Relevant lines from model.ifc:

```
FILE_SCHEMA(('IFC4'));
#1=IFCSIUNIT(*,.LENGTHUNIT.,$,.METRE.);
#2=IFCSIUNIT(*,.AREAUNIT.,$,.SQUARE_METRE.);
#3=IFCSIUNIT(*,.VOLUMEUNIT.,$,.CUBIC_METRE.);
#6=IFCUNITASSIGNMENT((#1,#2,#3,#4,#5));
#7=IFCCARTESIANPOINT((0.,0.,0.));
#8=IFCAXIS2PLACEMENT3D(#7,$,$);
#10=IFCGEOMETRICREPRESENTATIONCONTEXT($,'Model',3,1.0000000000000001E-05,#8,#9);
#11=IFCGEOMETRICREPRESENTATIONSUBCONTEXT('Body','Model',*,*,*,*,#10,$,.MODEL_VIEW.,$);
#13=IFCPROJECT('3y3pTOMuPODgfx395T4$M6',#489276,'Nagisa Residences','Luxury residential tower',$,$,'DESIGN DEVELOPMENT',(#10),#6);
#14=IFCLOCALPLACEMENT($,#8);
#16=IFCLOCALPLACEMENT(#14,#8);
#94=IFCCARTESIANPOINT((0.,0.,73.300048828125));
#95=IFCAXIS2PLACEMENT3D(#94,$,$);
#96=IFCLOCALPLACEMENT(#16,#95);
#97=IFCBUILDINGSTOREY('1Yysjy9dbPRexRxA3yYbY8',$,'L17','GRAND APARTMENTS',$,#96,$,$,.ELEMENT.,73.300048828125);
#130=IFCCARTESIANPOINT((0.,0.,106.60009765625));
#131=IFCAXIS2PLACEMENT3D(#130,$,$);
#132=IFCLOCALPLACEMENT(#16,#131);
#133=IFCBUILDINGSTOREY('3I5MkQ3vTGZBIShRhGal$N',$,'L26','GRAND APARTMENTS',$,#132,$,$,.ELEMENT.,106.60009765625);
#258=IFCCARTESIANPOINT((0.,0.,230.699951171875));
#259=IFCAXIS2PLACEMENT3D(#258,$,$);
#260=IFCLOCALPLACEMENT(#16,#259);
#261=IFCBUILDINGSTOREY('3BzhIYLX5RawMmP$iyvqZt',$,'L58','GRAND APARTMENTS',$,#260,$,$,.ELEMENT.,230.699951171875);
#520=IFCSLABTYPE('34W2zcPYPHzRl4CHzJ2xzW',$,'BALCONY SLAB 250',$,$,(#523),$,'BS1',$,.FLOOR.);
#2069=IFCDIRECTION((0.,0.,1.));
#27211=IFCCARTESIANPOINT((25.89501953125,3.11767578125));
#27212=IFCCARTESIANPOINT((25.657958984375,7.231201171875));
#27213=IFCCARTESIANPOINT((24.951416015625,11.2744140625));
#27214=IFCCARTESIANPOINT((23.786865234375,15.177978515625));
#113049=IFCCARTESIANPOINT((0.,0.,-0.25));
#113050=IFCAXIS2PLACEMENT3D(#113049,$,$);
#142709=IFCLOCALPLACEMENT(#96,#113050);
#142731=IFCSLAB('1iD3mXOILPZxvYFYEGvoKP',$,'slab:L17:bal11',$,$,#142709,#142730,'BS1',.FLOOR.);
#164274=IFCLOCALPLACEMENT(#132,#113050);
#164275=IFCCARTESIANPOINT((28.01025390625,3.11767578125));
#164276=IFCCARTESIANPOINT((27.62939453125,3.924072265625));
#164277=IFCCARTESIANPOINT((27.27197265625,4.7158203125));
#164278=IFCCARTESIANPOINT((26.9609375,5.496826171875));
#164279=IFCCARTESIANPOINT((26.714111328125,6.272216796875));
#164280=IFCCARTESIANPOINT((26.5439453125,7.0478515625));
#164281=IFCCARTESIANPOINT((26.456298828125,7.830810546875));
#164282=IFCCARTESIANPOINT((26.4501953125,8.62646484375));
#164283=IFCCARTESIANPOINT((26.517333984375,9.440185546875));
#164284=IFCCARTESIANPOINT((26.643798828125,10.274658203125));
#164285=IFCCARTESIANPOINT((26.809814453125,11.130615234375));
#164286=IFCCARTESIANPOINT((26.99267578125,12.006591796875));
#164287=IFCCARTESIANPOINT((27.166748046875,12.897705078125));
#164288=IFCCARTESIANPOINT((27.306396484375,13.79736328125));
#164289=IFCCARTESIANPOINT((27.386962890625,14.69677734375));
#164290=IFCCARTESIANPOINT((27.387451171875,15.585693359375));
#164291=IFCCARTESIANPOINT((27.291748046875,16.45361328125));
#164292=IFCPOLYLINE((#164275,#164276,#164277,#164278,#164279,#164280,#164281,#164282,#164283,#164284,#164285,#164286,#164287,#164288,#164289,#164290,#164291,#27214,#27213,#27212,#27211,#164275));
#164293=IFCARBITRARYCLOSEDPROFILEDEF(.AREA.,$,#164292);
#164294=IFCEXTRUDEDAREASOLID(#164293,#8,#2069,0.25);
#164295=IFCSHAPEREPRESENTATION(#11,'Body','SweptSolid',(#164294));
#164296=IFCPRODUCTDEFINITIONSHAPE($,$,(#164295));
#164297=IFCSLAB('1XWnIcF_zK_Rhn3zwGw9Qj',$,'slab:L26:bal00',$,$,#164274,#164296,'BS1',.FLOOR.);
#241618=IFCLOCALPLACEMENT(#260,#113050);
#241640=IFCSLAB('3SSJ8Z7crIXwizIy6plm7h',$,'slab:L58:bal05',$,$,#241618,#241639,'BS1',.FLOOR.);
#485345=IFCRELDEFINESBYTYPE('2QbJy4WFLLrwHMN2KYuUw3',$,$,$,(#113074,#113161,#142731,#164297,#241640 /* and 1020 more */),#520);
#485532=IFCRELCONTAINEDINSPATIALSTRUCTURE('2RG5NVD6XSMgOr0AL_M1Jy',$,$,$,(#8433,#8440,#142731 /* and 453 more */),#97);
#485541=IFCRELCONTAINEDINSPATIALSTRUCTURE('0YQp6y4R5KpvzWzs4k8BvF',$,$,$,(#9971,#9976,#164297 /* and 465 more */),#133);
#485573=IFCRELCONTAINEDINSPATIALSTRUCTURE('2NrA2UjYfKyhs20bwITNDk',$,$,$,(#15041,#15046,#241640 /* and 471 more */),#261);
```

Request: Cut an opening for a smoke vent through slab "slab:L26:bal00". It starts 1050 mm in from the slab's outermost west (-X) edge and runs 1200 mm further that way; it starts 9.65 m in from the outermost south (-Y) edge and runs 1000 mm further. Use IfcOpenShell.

```python
import numpy as np
import ifcopenshell
import ifcopenshell.api.feature
import ifcopenshell.api.geometry
import ifcopenshell.api.root
import ifcopenshell.geom
import ifcopenshell.util.placement
import ifcopenshell.util.representation
import ifcopenshell.util.shape
import ifcopenshell.util.unit

model = ifcopenshell.open("model.ifc")
unit_scale = ifcopenshell.util.unit.calculate_unit_scale(model)
settings = ifcopenshell.geom.settings()


def volume(element):
    """Net volume in cubic metres, openings subtracted."""
    shape = ifcopenshell.geom.create_shape(settings, element)
    return ifcopenshell.util.shape.get_volume(shape.geometry)


slab = model.by_guid("1XWnIcF_zK_Rhn3zwGw9Qj")
before = volume(slab)

# Extent in the slab's own axes, in metres. The edges named are its -X and -Y sides.
slab_shape = ifcopenshell.geom.create_shape(settings, slab)
vertices = ifcopenshell.util.shape.get_vertices(slab_shape.geometry)
x_min, y_min, bottom = vertices.min(axis=0)
top = vertices[:, 2].max()

opening = ifcopenshell.api.root.create_entity(model, ifc_class="IfcOpeningElement", name="Smoke vent opening", predefined_type="OPENING")
context = ifcopenshell.util.representation.get_context(model, "Model", "Body", "MODEL_VIEW")
width, depth = 1.2, 1
outline = [(0.0, 0.0), (width, 0.0), (width, depth), (0.0, depth), (0.0, 0.0)]
# Overshoot both faces by 50 mm so the cut is clean.
shape = ifcopenshell.api.geometry.add_slab_representation(
    model, context=context, depth=top - bottom + 0.1, polyline=outline
)
ifcopenshell.api.geometry.assign_representation(model, product=opening, representation=shape)

matrix = ifcopenshell.util.placement.get_local_placement(slab.ObjectPlacement)
matrix[:, 3] = matrix @ np.append(np.array([x_min + 1.05, y_min + 9.65, bottom - 0.05]) / unit_scale, 1.0)
ifcopenshell.api.geometry.edit_object_placement(model, product=opening, matrix=matrix, is_si=False)
ifcopenshell.api.feature.add_feature(model, feature=opening, element=slab)

after = volume(slab)

print(f"slab volume {before:.3f} -> {after:.3f} m3")

model.write("model_rev.ifc")
```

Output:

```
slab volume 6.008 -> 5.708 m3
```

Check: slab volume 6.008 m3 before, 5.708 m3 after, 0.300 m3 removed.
